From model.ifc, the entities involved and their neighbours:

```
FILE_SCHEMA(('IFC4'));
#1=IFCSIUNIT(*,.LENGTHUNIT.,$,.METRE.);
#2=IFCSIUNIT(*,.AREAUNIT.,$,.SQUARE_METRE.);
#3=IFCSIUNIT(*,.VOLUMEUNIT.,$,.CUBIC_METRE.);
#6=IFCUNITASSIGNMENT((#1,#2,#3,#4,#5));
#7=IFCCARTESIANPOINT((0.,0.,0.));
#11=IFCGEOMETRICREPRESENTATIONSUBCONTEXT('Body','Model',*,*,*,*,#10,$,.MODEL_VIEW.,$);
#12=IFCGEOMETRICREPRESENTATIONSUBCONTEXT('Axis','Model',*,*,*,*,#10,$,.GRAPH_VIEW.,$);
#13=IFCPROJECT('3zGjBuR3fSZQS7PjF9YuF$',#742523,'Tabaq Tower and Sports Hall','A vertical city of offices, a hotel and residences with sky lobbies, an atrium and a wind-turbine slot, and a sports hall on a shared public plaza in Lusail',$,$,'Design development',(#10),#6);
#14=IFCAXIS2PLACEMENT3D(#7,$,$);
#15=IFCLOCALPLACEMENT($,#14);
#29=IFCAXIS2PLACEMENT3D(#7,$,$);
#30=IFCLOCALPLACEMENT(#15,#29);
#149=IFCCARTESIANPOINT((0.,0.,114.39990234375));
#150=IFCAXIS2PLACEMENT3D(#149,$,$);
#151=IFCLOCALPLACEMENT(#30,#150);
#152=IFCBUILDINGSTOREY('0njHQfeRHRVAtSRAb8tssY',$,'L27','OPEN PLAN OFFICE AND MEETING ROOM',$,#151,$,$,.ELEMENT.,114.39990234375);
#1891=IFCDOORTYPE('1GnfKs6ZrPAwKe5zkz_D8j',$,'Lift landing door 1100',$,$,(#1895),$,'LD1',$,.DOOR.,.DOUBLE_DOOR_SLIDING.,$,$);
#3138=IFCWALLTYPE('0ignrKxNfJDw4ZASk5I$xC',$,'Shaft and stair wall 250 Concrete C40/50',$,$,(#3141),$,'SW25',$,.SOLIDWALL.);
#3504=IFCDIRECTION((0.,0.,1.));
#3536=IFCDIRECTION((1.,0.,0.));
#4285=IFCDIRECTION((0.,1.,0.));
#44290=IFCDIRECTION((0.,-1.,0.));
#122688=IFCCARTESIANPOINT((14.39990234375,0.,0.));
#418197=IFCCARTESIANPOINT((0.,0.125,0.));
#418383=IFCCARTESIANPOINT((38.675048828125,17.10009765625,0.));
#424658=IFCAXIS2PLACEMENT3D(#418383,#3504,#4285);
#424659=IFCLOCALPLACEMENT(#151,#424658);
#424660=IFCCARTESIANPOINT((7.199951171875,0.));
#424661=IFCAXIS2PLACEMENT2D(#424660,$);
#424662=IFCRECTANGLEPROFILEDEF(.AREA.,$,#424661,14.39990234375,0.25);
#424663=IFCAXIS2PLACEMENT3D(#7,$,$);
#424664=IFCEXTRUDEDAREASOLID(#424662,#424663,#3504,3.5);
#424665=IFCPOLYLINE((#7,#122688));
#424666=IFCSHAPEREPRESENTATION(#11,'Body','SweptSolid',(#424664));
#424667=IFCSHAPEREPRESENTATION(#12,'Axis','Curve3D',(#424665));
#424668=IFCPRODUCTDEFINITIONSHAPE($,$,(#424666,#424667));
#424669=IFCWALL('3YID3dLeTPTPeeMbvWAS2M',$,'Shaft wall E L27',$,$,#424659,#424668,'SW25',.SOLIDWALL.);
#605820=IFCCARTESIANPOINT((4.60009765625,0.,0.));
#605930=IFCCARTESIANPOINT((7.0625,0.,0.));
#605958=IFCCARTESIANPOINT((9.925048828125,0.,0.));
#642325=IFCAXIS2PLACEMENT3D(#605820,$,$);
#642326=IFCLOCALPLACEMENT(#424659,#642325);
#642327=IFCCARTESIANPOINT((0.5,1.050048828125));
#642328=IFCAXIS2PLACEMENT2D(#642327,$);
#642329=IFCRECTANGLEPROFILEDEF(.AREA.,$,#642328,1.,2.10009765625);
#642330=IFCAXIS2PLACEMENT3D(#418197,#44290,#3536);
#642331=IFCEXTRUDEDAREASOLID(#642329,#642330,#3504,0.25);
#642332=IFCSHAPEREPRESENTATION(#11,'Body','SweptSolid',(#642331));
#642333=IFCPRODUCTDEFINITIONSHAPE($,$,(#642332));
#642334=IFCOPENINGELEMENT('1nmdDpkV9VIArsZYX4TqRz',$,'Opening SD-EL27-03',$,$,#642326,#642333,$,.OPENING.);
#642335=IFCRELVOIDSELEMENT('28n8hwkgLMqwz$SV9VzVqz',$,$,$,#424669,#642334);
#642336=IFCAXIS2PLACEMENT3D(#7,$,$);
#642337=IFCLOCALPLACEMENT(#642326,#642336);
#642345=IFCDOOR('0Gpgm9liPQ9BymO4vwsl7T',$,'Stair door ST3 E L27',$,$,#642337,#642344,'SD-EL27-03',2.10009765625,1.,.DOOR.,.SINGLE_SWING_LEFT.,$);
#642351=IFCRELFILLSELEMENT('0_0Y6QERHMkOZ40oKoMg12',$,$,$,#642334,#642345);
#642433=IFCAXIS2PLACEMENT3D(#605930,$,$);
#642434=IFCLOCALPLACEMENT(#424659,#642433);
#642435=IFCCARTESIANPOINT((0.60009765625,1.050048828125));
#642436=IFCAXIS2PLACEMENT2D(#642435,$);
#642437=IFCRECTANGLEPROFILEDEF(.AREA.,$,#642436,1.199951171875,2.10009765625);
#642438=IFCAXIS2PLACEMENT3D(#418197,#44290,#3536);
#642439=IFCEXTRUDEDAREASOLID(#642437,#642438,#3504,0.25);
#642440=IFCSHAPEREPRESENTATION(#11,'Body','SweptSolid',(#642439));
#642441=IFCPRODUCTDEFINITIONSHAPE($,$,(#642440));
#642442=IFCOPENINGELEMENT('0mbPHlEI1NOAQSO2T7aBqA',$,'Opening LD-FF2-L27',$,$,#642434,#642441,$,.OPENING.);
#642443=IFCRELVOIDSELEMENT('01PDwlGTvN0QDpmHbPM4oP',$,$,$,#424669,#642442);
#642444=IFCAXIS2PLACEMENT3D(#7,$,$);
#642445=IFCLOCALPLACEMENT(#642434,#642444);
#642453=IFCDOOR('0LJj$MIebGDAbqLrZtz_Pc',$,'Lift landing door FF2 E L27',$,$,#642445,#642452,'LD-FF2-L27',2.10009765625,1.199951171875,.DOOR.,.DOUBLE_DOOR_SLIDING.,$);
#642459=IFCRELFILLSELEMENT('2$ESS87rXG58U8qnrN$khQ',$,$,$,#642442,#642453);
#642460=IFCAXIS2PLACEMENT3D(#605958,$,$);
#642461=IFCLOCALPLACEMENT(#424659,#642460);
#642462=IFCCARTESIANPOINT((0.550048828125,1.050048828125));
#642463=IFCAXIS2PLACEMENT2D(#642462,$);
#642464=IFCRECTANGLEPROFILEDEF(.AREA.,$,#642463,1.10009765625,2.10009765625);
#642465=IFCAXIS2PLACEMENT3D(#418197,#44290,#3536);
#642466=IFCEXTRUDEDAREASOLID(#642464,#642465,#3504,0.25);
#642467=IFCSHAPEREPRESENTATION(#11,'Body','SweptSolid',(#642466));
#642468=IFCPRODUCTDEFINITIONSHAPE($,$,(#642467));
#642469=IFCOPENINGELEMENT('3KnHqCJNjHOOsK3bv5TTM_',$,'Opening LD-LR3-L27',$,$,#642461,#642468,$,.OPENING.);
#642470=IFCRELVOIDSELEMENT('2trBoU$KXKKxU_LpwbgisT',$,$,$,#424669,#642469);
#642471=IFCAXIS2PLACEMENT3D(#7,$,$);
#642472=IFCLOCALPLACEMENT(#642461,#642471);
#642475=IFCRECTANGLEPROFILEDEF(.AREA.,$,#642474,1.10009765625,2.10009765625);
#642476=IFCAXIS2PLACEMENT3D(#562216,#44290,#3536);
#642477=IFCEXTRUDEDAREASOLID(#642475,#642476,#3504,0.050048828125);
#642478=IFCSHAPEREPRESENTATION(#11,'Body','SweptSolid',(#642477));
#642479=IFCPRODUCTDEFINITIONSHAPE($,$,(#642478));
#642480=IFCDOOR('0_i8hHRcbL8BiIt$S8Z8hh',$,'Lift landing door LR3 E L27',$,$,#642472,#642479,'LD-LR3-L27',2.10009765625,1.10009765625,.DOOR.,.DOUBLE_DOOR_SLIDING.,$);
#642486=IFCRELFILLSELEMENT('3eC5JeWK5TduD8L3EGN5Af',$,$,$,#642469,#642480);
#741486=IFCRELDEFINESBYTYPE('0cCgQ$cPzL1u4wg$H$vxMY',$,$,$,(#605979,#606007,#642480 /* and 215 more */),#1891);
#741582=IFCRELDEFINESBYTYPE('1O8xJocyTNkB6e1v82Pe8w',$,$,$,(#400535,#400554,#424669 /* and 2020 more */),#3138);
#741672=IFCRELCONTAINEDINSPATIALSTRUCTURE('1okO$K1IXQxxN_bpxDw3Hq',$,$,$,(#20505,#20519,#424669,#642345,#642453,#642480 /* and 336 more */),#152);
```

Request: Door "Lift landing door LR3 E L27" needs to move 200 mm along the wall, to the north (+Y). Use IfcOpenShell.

```python
import ifcopenshell
import ifcopenshell.api.geometry
import ifcopenshell.util.placement

model = ifcopenshell.open("model.ifc")

door = model.by_id(642480)
opening = door.FillsVoids[0].RelatingOpeningElement
wall = opening.VoidsElements[0].RelatingBuildingElement

wall_matrix = ifcopenshell.util.placement.get_local_placement(wall.ObjectPlacement)
shift = wall_matrix[:3, 0] * 0.2
before = ifcopenshell.util.placement.get_local_placement(door.ObjectPlacement)[:3, 3].copy()

# The door is placed relative to its opening, so it follows when the opening moves.
matrix = ifcopenshell.util.placement.get_local_placement(opening.ObjectPlacement)
matrix[:3, 3] += shift
ifcopenshell.api.geometry.edit_object_placement(
    model, product=opening, matrix=matrix, is_si=False, should_transform_children=True
)

after = ifcopenshell.util.placement.get_local_placement(door.ObjectPlacement)[:3, 3]
print("door moved by", (after - before).round(3) + 0.0)

model.write("model_rev.ifc")
```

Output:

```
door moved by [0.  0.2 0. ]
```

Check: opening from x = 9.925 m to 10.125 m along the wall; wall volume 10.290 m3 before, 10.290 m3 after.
